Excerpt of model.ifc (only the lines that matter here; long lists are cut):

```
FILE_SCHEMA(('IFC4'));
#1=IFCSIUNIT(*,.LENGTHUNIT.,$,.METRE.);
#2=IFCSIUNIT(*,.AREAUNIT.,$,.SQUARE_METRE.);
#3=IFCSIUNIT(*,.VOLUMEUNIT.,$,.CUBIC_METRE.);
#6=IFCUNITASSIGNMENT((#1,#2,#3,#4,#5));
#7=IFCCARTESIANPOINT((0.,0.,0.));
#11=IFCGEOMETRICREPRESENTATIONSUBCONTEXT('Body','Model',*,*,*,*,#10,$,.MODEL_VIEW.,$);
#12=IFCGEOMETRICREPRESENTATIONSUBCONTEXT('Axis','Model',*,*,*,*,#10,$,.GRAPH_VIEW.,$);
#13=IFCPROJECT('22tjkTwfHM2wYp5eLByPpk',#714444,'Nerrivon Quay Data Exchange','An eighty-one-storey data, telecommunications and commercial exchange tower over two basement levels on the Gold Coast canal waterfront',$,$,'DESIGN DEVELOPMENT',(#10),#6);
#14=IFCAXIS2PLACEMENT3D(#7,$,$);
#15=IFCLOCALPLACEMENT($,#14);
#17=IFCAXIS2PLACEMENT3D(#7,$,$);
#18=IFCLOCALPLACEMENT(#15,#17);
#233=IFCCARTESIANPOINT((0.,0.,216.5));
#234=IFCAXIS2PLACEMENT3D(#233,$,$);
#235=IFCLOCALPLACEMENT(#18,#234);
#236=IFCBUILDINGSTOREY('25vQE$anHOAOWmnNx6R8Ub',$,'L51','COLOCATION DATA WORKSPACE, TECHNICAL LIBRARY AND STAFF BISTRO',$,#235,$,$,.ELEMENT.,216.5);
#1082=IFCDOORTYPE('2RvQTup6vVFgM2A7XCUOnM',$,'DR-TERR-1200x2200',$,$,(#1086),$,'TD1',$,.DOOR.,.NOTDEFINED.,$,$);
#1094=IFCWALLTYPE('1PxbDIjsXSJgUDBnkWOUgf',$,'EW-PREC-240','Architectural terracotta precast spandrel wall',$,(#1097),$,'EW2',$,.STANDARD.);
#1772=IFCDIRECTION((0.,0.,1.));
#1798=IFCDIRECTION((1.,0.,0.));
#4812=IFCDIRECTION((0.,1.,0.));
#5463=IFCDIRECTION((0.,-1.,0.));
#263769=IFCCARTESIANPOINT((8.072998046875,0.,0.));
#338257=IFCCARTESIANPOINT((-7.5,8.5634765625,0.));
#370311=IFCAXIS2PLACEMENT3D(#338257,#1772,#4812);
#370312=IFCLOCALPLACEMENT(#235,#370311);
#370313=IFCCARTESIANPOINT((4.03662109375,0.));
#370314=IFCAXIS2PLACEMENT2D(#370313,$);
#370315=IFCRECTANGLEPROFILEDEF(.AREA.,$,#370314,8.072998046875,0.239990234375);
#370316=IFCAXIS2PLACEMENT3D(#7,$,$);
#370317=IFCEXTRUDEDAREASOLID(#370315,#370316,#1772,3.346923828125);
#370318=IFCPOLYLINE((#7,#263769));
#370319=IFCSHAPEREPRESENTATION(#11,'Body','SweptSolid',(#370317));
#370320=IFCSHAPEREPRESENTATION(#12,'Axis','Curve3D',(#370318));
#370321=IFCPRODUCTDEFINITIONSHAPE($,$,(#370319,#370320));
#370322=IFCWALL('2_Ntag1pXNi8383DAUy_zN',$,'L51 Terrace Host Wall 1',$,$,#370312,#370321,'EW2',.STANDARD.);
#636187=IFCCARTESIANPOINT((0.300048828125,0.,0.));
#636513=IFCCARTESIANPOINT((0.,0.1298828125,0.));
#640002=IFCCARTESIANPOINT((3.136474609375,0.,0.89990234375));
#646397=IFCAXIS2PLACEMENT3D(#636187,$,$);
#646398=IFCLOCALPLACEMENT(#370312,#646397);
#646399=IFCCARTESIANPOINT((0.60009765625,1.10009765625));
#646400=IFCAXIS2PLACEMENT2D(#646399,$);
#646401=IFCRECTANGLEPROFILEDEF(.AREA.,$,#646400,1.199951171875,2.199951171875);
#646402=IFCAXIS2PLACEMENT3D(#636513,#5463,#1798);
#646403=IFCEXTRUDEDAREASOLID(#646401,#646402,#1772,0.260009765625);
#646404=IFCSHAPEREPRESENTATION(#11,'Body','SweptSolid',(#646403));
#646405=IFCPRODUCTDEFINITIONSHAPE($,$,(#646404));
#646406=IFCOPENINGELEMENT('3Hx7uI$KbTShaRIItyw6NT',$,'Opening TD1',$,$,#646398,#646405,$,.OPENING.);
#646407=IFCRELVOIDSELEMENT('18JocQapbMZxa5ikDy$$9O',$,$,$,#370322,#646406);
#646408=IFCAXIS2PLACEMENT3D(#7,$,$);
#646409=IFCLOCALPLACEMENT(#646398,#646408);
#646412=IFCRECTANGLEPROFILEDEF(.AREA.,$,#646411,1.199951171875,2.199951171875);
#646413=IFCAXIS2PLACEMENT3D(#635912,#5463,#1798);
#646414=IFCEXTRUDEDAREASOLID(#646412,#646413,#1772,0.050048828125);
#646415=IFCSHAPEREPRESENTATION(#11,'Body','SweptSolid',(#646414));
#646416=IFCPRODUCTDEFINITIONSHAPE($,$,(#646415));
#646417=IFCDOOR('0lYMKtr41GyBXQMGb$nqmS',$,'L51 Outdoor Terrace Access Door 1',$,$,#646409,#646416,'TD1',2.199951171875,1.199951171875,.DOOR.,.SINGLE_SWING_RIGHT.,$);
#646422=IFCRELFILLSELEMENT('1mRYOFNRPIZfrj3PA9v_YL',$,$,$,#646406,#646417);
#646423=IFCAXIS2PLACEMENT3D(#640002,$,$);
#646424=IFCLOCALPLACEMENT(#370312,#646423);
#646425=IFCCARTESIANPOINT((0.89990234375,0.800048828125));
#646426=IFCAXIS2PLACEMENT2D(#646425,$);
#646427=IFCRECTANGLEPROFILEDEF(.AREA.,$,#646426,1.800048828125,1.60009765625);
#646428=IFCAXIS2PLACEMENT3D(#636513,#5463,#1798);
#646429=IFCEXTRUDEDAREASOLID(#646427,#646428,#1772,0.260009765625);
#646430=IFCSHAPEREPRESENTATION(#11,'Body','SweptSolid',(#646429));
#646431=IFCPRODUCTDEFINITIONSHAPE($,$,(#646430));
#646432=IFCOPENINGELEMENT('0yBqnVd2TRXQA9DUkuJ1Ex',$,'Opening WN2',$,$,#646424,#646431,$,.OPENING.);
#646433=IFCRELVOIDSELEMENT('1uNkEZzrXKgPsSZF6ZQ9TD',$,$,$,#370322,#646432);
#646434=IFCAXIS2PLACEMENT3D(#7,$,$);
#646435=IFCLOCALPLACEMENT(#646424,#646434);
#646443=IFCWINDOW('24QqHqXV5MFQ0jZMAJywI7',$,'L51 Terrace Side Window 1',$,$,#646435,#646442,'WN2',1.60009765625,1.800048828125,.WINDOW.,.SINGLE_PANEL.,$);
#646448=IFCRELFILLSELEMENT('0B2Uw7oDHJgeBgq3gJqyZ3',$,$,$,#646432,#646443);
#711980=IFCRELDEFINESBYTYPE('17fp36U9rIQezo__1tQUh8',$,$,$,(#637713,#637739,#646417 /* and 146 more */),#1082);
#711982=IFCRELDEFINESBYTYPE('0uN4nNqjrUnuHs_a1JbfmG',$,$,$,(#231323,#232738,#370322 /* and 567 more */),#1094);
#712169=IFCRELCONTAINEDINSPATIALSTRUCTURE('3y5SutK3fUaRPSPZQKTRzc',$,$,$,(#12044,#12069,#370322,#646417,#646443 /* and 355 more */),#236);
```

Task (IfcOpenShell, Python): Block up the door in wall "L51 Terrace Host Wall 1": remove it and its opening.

```python
import ifcopenshell
import ifcopenshell.api.feature
import ifcopenshell.api.root
import ifcopenshell.geom
import ifcopenshell.util.shape

model = ifcopenshell.open("model.ifc")
settings = ifcopenshell.geom.settings()


def volume(element):
    """Net volume in cubic metres, openings subtracted."""
    shape = ifcopenshell.geom.create_shape(settings, element)
    return ifcopenshell.util.shape.get_volume(shape.geometry)


door = model.by_guid("0lYMKtr41GyBXQMGb$nqmS")
opening = door.FillsVoids[0].RelatingOpeningElement
wall = opening.VoidsElements[0].RelatingBuildingElement
before = volume(wall)

ifcopenshell.api.root.remove_product(model, product=door)
ifcopenshell.api.feature.remove_feature(model, feature=opening)

after = volume(wall)

print(f"wall volume {before:.3f} -> {after:.3f} m3")

model.write("model_updated.ifc")
```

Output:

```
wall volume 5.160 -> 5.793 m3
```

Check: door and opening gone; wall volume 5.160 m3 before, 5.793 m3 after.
